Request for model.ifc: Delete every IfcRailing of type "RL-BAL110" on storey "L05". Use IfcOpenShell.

First a look at what the model holds.

```python
import ifcopenshell
import ifcopenshell.util.element

model = ifcopenshell.open("model.ifc")
print(model.schema)
storey = next(s for s in model.by_type("IfcBuildingStorey") if s.Name == "L05")
railings = [e for e in ifcopenshell.util.element.get_decomposition(storey) if e.is_a("IfcRailing")]
seen = {}
for e in railings:
    element_type = ifcopenshell.util.element.get_type(e)
    name = element_type.Name if element_type not in (None, e) else None
    seen[name] = seen.get(name, 0) + 1
for name, count in sorted(seen.items(), key=str):
    print(count, "x", name)
```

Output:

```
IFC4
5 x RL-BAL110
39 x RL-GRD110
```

```python
import ifcopenshell
import ifcopenshell.api.root
import ifcopenshell.util.element

model = ifcopenshell.open("model.ifc")

storey = next(s for s in model.by_type("IfcBuildingStorey") if s.Name == "L05")
railings = [e for e in ifcopenshell.util.element.get_decomposition(storey) if e.is_a("IfcRailing")]
targets = [e for e in railings if (t := ifcopenshell.util.element.get_type(e)) not in (None, e) and t.Name == "RL-BAL110"]

for e in targets:
    ifcopenshell.api.root.remove_product(model, product=e)
print(len(targets), "removed")

model.write("model-out.ifc")
```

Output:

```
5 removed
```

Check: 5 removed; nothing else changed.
